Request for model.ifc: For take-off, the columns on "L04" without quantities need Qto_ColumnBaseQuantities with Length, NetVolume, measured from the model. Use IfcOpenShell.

First a look at what the model holds.

```python
import ifcopenshell
import ifcopenshell.util.element
import ifcopenshell.util.unit

model = ifcopenshell.open("model.ifc")
print(model.schema)
for unit_type in ("LENGTHUNIT", "AREAUNIT", "VOLUMEUNIT"):
    print(unit_type, ifcopenshell.util.unit.calculate_unit_scale(model, unit_type))
storey = next(s for s in model.by_type("IfcBuildingStorey") if s.Name == "L04")
columns = [e for e in ifcopenshell.util.element.get_decomposition(storey) if e.is_a("IfcColumn")]
for e in sorted(columns, key=lambda e: e.id()):
    print(e.id(), e.is_a(), e.Name, list(ifcopenshell.util.element.get_psets(e, qtos_only=True)), sep=" | ")
```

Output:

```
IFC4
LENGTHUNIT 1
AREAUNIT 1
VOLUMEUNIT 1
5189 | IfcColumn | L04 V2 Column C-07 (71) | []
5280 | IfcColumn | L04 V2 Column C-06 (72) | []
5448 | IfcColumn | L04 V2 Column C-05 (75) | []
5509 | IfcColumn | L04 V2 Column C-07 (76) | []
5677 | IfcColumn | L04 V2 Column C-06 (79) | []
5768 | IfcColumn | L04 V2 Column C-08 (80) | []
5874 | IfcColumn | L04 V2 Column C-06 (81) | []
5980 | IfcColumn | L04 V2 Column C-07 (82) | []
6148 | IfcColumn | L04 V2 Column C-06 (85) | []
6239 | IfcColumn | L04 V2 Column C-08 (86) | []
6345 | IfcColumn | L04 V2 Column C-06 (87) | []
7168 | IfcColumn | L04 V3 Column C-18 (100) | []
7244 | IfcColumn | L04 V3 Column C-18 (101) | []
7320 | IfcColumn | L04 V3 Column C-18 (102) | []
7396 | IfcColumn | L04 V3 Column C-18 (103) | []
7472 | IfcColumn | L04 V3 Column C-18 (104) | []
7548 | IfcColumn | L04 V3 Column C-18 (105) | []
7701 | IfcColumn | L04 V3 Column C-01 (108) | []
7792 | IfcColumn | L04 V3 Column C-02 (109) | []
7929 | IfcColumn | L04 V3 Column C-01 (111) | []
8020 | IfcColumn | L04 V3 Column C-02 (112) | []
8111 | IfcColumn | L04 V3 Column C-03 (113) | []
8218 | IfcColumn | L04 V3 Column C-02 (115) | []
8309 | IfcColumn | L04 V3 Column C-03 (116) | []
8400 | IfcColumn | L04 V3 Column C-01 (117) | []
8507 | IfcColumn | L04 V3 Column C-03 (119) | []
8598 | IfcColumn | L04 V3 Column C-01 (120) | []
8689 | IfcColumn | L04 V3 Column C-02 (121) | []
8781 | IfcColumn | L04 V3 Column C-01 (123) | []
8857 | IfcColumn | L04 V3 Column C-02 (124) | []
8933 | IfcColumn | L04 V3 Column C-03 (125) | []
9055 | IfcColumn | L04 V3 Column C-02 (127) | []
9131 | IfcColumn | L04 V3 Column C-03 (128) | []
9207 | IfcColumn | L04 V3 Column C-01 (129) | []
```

```python
import ifcopenshell
import ifcopenshell.api.pset
import ifcopenshell.geom
import ifcopenshell.util.element
import ifcopenshell.util.shape
import ifcopenshell.util.unit

model = ifcopenshell.open("model.ifc")
unit_scale = ifcopenshell.util.unit.calculate_unit_scale(model)
volume_scale = ifcopenshell.util.unit.calculate_unit_scale(model, "VOLUMEUNIT")
settings = ifcopenshell.geom.settings()

storey = next(s for s in model.by_type("IfcBuildingStorey") if s.Name == "L04")
columns = [e for e in ifcopenshell.util.element.get_decomposition(storey) if e.is_a("IfcColumn")]

for e in sorted(columns, key=lambda e: e.id()):
    if ifcopenshell.util.element.get_psets(e, qtos_only=True, should_inherit=False):
        continue
    # Geometry comes back in metres, in the element's own axes.
    shape = ifcopenshell.geom.create_shape(settings, e)
    values = {
        "Length": ifcopenshell.util.shape.get_z(shape.geometry) / unit_scale,
        "NetVolume": ifcopenshell.util.shape.get_volume(shape.geometry) / volume_scale,
    }
    qto = ifcopenshell.api.pset.add_qto(model, product=e, name="Qto_ColumnBaseQuantities")
    ifcopenshell.api.pset.edit_qto(model, qto=qto, properties=values)
    print(e.id(), {k: round(v, 3) for k, v in values.items()})

model.write("model_updated.ifc")
```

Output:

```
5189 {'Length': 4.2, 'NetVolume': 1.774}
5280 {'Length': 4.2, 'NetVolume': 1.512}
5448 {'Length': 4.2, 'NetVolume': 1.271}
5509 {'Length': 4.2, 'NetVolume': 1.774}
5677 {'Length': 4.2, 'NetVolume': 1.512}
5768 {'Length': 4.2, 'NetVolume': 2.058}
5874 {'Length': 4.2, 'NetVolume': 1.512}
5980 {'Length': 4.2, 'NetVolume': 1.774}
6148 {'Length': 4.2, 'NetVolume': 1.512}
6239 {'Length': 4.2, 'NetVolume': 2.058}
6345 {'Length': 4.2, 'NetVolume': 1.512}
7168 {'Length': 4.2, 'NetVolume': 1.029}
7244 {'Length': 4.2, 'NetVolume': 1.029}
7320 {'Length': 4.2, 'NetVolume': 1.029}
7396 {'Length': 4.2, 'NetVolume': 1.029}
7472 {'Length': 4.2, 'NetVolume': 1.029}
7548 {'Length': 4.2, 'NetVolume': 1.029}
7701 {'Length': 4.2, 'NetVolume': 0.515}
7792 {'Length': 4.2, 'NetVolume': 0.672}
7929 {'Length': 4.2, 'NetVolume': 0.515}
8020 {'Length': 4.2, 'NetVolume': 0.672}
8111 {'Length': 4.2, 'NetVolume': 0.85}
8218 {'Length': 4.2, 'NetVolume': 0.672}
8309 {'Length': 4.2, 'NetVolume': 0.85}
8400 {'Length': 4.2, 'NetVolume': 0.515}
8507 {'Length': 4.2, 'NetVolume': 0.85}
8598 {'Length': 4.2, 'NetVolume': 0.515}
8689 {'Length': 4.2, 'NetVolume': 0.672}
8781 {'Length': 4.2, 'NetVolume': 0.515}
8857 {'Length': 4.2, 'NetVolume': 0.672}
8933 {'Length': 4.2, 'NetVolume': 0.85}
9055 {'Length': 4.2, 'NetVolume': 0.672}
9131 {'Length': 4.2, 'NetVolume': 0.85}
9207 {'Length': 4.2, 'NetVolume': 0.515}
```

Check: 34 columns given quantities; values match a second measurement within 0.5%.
